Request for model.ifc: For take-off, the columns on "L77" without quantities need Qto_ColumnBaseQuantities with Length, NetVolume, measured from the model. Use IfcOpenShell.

First a look at what the model holds.

```python
import ifcopenshell
import ifcopenshell.util.element
import ifcopenshell.util.unit

model = ifcopenshell.open("model.ifc")
print(model.schema)
for unit_type in ("LENGTHUNIT", "AREAUNIT", "VOLUMEUNIT"):
    print(unit_type, ifcopenshell.util.unit.calculate_unit_scale(model, unit_type))
storey = next(s for s in model.by_type("IfcBuildingStorey") if s.Name == "L77")
columns = [e for e in ifcopenshell.util.element.get_decomposition(storey) if e.is_a("IfcColumn")]
for e in sorted(columns, key=lambda e: e.id()):
    print(e.id(), e.is_a(), e.Name, list(ifcopenshell.util.element.get_psets(e, qtos_only=True)), sep=" | ")
```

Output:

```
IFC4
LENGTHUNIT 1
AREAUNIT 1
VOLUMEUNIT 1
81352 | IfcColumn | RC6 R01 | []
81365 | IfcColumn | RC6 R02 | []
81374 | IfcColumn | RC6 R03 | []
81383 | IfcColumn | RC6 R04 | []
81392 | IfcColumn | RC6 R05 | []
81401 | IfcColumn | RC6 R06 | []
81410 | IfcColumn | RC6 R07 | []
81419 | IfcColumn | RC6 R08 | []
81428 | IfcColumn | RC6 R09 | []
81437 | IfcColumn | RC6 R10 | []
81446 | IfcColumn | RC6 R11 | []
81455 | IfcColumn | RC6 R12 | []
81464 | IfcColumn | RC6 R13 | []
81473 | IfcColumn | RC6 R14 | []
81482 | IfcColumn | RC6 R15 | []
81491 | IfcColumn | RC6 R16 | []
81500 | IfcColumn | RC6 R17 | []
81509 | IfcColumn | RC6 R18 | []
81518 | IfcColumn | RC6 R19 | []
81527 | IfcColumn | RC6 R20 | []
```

```python
import ifcopenshell
import ifcopenshell.api.pset
import ifcopenshell.geom
import ifcopenshell.util.element
import ifcopenshell.util.shape
import ifcopenshell.util.unit

model = ifcopenshell.open("model.ifc")
unit_scale = ifcopenshell.util.unit.calculate_unit_scale(model)
volume_scale = ifcopenshell.util.unit.calculate_unit_scale(model, "VOLUMEUNIT")
settings = ifcopenshell.geom.settings()

storey = next(s for s in model.by_type("IfcBuildingStorey") if s.Name == "L77")
columns = [e for e in ifcopenshell.util.element.get_decomposition(storey) if e.is_a("IfcColumn")]

for e in sorted(columns, key=lambda e: e.id()):
    if ifcopenshell.util.element.get_psets(e, qtos_only=True, should_inherit=False):
        continue
    # Geometry comes back in metres, in the element's own axes.
    shape = ifcopenshell.geom.create_shape(settings, e)
    values = {
        "Length": ifcopenshell.util.shape.get_z(shape.geometry) / unit_scale,
        "NetVolume": ifcopenshell.util.shape.get_volume(shape.geometry) / volume_scale,
    }
    qto = ifcopenshell.api.pset.add_qto(model, product=e, name="Qto_ColumnBaseQuantities")
    ifcopenshell.api.pset.edit_qto(model, qto=qto, properties=values)
    print(e.id(), {k: round(v, 3) for k, v in values.items()})

model.write("model-out.ifc")
```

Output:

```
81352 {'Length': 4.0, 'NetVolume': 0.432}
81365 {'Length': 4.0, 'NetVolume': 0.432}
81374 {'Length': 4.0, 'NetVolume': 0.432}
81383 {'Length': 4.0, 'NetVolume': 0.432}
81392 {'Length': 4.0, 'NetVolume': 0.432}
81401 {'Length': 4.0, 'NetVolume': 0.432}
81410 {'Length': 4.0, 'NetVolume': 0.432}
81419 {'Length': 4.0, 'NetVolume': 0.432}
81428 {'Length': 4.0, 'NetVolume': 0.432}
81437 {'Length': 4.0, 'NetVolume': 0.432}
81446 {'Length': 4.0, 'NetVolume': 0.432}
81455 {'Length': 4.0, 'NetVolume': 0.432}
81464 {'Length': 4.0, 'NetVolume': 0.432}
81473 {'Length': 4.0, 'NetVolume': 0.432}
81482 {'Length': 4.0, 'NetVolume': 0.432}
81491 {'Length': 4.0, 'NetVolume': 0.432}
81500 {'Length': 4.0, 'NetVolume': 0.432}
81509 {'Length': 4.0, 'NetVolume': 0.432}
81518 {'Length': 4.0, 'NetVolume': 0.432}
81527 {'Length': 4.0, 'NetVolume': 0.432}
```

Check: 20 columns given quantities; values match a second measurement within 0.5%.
